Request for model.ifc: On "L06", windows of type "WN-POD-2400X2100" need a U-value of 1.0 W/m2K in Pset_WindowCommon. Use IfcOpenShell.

First a look at what the model holds.

```python
import ifcopenshell
import ifcopenshell.util.element

model = ifcopenshell.open("model.ifc")
print(model.schema)
storey = next(s for s in model.by_type("IfcBuildingStorey") if s.Name == "L06")
windows = [e for e in ifcopenshell.util.element.get_decomposition(storey) if e.is_a("IfcWindow")]
seen = {}
for e in windows:
    element_type = ifcopenshell.util.element.get_type(e)
    key = (element_type.Name if element_type != e and element_type else None, ifcopenshell.util.element.get_pset(e, "Pset_WindowCommon", "ThermalTransmittance"))
    seen[key] = seen.get(key, 0) + 1
for (name, value), count in sorted(seen.items(), key=str):
    print(count, "x", name, "|", value)
```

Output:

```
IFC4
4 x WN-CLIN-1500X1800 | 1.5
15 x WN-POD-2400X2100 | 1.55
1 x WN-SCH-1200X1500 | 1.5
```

```python
import ifcopenshell
import ifcopenshell.api.pset
import ifcopenshell.util.element

model = ifcopenshell.open("model.ifc")

storey = next(s for s in model.by_type("IfcBuildingStorey") if s.Name == "L06")
windows = [e for e in ifcopenshell.util.element.get_decomposition(storey) if e.is_a("IfcWindow")]

count = 0
for e in windows:
    element_type = ifcopenshell.util.element.get_type(e)
    if element_type in (None, e) or element_type.Name != "WN-POD-2400X2100":
        continue
    found = ifcopenshell.util.element.get_pset(e, "Pset_WindowCommon", should_inherit=False)
    if found:
        pset = model.by_id(found["id"])
        if len(ifcopenshell.util.element.get_elements_by_pset(pset)) > 1:
            pset = ifcopenshell.api.pset.unshare_pset(model, products=[e], pset=pset)[0]
    else:
        pset = ifcopenshell.api.pset.add_pset(model, product=e, name="Pset_WindowCommon")
    ifcopenshell.api.pset.edit_pset(model, pset=pset, properties={"ThermalTransmittance": 1.0})
    count += 1

print(count, "windows updated")

model.write("model_edited.ifc")
```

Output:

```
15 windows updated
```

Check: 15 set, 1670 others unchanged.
